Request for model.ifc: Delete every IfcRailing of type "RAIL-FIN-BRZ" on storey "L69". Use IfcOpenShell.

First a look at what the model holds.

```python
import ifcopenshell
import ifcopenshell.util.element

model = ifcopenshell.open("model.ifc")
print(model.schema)
storey = next(s for s in model.by_type("IfcBuildingStorey") if s.Name == "L69")
railings = [e for e in ifcopenshell.util.element.get_decomposition(storey) if e.is_a("IfcRailing")]
seen = {}
for e in railings:
    element_type = ifcopenshell.util.element.get_type(e)
    name = element_type.Name if element_type not in (None, e) else None
    seen[name] = seen.get(name, 0) + 1
for name, count in sorted(seen.items(), key=str):
    print(count, "x", name)
```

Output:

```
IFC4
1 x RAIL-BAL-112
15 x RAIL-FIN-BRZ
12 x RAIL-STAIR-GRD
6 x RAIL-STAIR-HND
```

```python
import ifcopenshell
import ifcopenshell.api.root
import ifcopenshell.util.element

model = ifcopenshell.open("model.ifc")

storey = next(s for s in model.by_type("IfcBuildingStorey") if s.Name == "L69")
railings = [e for e in ifcopenshell.util.element.get_decomposition(storey) if e.is_a("IfcRailing")]
targets = [e for e in railings if (t := ifcopenshell.util.element.get_type(e)) not in (None, e) and t.Name == "RAIL-FIN-BRZ"]

for e in targets:
    ifcopenshell.api.root.remove_product(model, product=e)
print(len(targets), "removed")

model.write("model_v2.ifc")
```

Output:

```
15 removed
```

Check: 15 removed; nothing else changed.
